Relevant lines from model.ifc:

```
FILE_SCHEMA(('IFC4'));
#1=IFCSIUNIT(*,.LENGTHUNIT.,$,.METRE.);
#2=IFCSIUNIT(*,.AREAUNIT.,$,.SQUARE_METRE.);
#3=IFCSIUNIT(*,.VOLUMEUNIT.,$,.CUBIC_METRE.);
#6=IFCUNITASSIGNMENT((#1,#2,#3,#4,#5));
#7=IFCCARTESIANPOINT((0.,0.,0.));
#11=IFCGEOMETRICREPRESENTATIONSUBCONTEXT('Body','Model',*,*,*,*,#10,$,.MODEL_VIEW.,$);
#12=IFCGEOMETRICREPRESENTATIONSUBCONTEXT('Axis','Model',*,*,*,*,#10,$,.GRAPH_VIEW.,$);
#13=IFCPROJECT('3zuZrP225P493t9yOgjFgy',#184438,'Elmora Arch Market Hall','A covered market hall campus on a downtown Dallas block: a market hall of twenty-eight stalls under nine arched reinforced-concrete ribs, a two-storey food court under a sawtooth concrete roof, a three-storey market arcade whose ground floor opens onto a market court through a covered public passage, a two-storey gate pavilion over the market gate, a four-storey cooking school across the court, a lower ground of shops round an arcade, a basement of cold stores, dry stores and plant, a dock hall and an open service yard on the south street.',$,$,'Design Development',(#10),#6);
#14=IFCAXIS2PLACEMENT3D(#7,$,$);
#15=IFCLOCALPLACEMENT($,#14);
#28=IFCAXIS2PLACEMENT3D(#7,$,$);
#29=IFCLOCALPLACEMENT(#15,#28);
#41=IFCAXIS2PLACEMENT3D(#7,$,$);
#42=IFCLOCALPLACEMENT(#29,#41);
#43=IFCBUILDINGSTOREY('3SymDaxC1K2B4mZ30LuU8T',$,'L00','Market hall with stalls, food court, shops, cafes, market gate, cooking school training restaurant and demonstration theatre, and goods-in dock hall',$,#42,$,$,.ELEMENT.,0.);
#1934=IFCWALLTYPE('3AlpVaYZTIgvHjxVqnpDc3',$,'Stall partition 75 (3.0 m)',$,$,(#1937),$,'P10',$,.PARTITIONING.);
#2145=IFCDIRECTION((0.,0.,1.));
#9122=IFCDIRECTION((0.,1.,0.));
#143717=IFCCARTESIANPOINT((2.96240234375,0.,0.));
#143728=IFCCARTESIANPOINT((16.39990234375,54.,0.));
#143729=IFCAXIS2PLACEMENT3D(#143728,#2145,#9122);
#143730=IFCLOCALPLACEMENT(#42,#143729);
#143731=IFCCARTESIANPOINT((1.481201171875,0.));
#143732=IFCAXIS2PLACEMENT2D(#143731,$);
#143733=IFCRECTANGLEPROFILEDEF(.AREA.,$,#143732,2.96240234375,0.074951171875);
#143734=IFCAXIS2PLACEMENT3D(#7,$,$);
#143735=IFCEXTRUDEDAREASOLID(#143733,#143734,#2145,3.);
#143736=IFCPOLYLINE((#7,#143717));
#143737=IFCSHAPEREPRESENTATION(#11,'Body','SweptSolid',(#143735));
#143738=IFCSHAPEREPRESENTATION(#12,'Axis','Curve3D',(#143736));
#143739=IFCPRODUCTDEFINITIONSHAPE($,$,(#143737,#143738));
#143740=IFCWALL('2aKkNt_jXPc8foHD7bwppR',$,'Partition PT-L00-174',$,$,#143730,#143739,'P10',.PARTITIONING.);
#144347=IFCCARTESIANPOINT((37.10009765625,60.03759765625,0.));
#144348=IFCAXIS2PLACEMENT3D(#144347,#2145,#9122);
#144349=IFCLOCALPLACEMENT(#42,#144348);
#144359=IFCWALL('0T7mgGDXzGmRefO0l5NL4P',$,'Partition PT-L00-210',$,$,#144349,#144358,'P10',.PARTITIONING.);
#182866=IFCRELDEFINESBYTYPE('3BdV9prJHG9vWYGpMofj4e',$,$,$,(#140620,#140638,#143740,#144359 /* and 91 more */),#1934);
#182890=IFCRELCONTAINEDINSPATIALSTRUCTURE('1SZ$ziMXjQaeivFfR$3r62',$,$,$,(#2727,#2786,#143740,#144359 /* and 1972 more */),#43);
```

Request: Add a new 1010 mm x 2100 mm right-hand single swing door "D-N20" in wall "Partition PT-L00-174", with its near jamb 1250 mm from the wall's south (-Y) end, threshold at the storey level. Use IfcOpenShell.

```python
import numpy as np
import ifcopenshell
import ifcopenshell.api.feature
import ifcopenshell.api.geometry
import ifcopenshell.api.root
import ifcopenshell.api.spatial
import ifcopenshell.geom
import ifcopenshell.util.element
import ifcopenshell.util.placement
import ifcopenshell.util.representation
import ifcopenshell.util.shape
import ifcopenshell.util.unit

model = ifcopenshell.open("model.ifc")
unit_scale = ifcopenshell.util.unit.calculate_unit_scale(model)
settings = ifcopenshell.geom.settings()


def volume(element):
    """Net volume in cubic metres, openings subtracted."""
    shape = ifcopenshell.geom.create_shape(settings, element)
    return ifcopenshell.util.shape.get_volume(shape.geometry)


wall = model.by_guid("2aKkNt_jXPc8foHD7bwppR")
storey = ifcopenshell.util.element.get_container(wall, ifc_class="IfcBuildingStorey")
context = ifcopenshell.util.representation.get_context(model, "Model", "Body", "MODEL_VIEW")
before = volume(wall)

width, height, from_end, sill = 1.01, 2.1, 1.25, 0.0  # metres

# The wall runs along its own X axis, and the end named is its -X end.
wall_shape = ifcopenshell.geom.create_shape(settings, wall)
x, y, z = ifcopenshell.util.shape.get_vertices(wall_shape.geometry).T
start = x.min() + from_end
face, thickness = float(y.min()), float(y.max() - y.min())
wall_matrix = ifcopenshell.util.placement.get_local_placement(wall.ObjectPlacement)
level = ifcopenshell.util.placement.get_local_placement(storey.ObjectPlacement)[2, 3]


def in_wall(x, y):
    """Placement at x, y metres in the wall's axes, at sill height."""
    matrix = wall_matrix.copy()
    matrix[:, 3] = wall_matrix @ np.array([x / unit_scale, y / unit_scale, 0.0, 1.0])
    matrix[2, 3] = level + sill / unit_scale
    return matrix


# Opening: a box that overshoots both wall faces by 50 mm.
opening = ifcopenshell.api.root.create_entity(model, ifc_class="IfcOpeningElement", predefined_type="OPENING")
box = ifcopenshell.api.geometry.add_wall_representation(
    model, context=context, length=width, height=height, thickness=thickness + 0.1
)
ifcopenshell.api.geometry.assign_representation(model, product=opening, representation=box)
ifcopenshell.api.geometry.edit_object_placement(model, product=opening, matrix=in_wall(start, face - 0.05), is_si=False)
ifcopenshell.api.feature.add_feature(model, feature=opening, element=wall)

door = ifcopenshell.api.root.create_entity(model, ifc_class="IfcDoor", name="D-N20", predefined_type="DOOR")
door.OverallWidth, door.OverallHeight = width / unit_scale, height / unit_scale
door.OperationType = "SINGLE_SWING_RIGHT"
body = ifcopenshell.api.geometry.add_door_representation(
    model,
    context=context,
    overall_width=door.OverallWidth,
    overall_height=door.OverallHeight,
    operation_type="SINGLE_SWING_RIGHT",
    lining_properties={"LiningDepth": thickness / unit_scale, "ThresholdDepth": thickness / unit_scale},
)
ifcopenshell.api.geometry.assign_representation(model, product=door, representation=body)
ifcopenshell.api.spatial.assign_container(model, products=[door], relating_structure=storey)
ifcopenshell.api.feature.add_filling(model, opening=opening, element=door)

# The lining spans the wall, so the door starts at the wall face.
ifcopenshell.api.geometry.edit_object_placement(model, product=door, matrix=in_wall(start, face), is_si=False)

after = volume(wall)

print(f"wall volume {before:.3f} -> {after:.3f} m3")

model.write("model-out.ifc")
```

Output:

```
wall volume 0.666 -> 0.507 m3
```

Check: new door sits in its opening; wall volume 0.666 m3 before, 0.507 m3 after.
